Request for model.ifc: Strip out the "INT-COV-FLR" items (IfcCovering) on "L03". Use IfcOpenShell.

First a look at what the model holds.

```python
import ifcopenshell
import ifcopenshell.util.element

model = ifcopenshell.open("model.ifc")
print(model.schema)
storey = next(s for s in model.by_type("IfcBuildingStorey") if s.Name == "L03")
coverings = [e for e in ifcopenshell.util.element.get_decomposition(storey) if e.is_a("IfcCovering")]
seen = {}
for e in coverings:
    element_type = ifcopenshell.util.element.get_type(e)
    name = element_type.Name if element_type not in (None, e) else None
    seen[name] = seen.get(name, 0) + 1
for name, count in sorted(seen.items(), key=str):
    print(count, "x", name)
```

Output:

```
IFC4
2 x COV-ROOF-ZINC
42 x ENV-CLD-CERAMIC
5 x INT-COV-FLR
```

```python
import ifcopenshell
import ifcopenshell.api.root
import ifcopenshell.util.element

model = ifcopenshell.open("model.ifc")

storey = next(s for s in model.by_type("IfcBuildingStorey") if s.Name == "L03")
coverings = [e for e in ifcopenshell.util.element.get_decomposition(storey) if e.is_a("IfcCovering")]
targets = [e for e in coverings if (t := ifcopenshell.util.element.get_type(e)) not in (None, e) and t.Name == "INT-COV-FLR"]

for e in targets:
    ifcopenshell.api.root.remove_product(model, product=e)
print(len(targets), "removed")

model.write("model_updated.ifc")
```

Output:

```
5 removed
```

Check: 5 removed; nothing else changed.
